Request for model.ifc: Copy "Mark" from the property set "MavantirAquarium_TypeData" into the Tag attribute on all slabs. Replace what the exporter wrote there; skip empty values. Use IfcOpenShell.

First a look at what the model holds.

```python
import ifcopenshell
import ifcopenshell.util.element

model = ifcopenshell.open("model.ifc")
print(model.schema)
slabs = model.by_type("IfcSlab")
print(len(slabs), "slabs")
for e in slabs[:8]:
    source = ifcopenshell.util.element.get_pset(e, "MavantirAquarium_TypeData", "Mark")
    target = e.Tag
    print(e.id(), repr(source), repr(target), sep=" | ")
```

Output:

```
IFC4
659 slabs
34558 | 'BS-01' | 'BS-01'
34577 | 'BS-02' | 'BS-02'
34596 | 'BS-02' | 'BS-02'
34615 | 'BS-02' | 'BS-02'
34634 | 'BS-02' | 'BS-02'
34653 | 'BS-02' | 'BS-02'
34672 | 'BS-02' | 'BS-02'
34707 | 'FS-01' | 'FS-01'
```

```python
import ifcopenshell
import ifcopenshell.util.element

model = ifcopenshell.open("model.ifc")

count = 0
for e in model.by_type("IfcSlab"):
    value = ifcopenshell.util.element.get_pset(e, "MavantirAquarium_TypeData", "Mark")
    current = e.Tag
    if not value or not value.strip() or current == value:
        continue
    e.Tag = value
    count += 1

print(count, "slabs updated")

model.write("model-out.ifc")
```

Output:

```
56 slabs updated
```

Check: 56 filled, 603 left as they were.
